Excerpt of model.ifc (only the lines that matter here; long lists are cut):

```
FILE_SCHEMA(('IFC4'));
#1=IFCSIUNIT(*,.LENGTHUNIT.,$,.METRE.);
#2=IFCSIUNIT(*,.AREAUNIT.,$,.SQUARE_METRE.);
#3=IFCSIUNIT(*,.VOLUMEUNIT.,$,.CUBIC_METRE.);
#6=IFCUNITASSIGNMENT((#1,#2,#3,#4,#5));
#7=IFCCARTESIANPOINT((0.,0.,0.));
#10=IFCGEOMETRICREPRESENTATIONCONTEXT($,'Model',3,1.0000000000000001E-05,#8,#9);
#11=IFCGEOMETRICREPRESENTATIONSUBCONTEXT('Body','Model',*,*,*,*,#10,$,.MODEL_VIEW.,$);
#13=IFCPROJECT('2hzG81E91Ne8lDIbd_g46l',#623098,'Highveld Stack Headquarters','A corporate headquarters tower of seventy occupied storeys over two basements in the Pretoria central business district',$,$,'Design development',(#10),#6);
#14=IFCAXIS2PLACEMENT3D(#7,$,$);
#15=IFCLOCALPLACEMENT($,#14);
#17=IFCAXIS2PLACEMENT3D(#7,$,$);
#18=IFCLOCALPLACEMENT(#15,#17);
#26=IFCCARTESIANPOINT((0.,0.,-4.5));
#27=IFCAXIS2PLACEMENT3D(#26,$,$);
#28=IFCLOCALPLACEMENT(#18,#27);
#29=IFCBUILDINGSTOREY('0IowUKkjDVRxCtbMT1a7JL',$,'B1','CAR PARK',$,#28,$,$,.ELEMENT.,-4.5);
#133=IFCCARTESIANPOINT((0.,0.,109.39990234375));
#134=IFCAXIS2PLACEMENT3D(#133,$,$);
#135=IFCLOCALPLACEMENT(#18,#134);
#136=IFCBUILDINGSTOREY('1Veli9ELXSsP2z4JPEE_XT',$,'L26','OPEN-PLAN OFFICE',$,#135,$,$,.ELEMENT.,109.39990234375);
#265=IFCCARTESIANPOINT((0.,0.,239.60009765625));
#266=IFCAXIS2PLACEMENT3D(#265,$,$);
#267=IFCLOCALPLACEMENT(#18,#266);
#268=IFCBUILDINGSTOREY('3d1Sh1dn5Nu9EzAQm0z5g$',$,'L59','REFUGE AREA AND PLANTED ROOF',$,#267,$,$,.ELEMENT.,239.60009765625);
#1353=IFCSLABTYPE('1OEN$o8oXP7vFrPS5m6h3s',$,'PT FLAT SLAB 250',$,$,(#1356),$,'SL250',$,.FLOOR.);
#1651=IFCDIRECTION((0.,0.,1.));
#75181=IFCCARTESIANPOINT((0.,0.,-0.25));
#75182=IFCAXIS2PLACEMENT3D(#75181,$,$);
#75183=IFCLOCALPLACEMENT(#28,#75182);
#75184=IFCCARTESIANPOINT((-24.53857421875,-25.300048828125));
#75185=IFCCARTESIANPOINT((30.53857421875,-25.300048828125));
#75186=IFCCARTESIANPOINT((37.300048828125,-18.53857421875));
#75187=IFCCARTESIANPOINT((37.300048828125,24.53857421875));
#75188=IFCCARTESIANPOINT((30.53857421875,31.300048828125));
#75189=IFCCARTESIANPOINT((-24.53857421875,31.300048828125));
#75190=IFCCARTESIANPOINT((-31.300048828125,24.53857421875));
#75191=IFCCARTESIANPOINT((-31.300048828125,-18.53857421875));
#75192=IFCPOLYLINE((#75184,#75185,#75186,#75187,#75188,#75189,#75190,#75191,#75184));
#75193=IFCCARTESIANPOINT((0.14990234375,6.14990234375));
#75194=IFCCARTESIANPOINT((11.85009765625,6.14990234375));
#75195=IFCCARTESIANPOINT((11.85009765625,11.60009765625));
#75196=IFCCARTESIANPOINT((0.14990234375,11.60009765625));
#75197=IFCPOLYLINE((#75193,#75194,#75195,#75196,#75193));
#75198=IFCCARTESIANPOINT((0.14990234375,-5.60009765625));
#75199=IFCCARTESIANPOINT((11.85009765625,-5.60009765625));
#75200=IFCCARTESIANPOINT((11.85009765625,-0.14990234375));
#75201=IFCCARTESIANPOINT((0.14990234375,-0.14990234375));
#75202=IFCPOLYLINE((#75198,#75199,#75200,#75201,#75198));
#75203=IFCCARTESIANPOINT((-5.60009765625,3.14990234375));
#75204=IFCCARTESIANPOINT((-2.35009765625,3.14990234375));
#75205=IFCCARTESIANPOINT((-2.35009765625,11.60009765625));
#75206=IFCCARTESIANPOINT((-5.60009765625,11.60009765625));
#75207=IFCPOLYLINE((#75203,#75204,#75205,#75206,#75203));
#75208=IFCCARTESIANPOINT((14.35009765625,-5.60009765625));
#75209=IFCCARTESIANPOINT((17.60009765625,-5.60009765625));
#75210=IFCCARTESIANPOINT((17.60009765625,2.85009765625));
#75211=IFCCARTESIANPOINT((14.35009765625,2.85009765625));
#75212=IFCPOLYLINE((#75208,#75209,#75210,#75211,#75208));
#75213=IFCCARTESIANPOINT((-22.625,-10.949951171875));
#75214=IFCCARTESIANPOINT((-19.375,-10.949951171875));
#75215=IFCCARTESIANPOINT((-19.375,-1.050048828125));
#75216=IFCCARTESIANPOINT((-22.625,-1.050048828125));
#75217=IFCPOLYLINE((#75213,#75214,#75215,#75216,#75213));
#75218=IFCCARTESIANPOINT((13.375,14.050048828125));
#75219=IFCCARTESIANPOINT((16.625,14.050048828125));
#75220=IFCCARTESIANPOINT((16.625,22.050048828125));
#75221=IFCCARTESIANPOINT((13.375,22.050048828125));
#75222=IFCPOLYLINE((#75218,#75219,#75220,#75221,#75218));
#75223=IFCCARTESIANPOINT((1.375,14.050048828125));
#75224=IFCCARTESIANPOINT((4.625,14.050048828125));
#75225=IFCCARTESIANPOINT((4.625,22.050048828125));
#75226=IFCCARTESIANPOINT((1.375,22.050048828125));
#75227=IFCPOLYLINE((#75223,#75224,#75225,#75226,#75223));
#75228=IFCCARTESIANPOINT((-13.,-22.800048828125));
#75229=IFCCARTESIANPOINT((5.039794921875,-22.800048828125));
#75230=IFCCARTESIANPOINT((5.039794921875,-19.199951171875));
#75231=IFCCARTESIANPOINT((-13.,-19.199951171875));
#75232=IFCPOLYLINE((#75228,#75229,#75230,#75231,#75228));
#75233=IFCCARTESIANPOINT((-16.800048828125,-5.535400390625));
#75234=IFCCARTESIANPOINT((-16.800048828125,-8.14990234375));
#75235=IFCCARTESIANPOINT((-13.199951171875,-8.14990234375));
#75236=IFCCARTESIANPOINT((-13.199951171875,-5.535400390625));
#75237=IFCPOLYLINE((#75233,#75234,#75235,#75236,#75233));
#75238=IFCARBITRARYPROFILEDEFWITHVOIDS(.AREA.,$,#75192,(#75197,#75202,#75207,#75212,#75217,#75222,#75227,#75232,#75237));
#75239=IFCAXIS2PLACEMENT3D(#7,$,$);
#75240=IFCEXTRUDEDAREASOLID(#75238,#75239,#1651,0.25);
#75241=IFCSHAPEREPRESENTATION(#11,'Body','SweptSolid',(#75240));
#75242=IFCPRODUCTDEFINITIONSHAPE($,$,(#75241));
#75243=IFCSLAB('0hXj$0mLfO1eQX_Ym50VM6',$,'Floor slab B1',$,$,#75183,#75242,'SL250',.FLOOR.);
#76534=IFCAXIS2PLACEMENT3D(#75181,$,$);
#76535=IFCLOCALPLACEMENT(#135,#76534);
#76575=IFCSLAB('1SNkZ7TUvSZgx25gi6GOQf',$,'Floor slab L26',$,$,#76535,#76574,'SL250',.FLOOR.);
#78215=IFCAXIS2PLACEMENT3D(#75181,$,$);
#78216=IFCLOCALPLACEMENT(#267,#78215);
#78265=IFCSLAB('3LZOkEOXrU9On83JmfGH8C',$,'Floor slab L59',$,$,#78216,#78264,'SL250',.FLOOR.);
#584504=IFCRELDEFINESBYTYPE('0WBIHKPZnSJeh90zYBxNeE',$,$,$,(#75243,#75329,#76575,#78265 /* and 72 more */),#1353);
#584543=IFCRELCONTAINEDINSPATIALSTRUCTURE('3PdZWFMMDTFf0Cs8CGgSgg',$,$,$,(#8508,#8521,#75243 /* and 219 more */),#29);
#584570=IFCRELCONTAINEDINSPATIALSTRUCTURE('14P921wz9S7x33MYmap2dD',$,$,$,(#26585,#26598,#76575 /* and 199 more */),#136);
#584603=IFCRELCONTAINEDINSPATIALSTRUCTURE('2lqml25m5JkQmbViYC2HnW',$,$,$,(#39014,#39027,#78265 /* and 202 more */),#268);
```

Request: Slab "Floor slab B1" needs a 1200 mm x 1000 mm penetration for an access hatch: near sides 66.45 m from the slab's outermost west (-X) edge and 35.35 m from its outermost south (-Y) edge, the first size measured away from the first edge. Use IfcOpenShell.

```python
import numpy as np
import ifcopenshell
import ifcopenshell.api.feature
import ifcopenshell.api.geometry
import ifcopenshell.api.root
import ifcopenshell.geom
import ifcopenshell.util.placement
import ifcopenshell.util.representation
import ifcopenshell.util.shape
import ifcopenshell.util.unit

model = ifcopenshell.open("model.ifc")
unit_scale = ifcopenshell.util.unit.calculate_unit_scale(model)
settings = ifcopenshell.geom.settings()


def volume(element):
    """Net volume in cubic metres, openings subtracted."""
    shape = ifcopenshell.geom.create_shape(settings, element)
    return ifcopenshell.util.shape.get_volume(shape.geometry)


slab = model.by_guid("0hXj$0mLfO1eQX_Ym50VM6")
before = volume(slab)

# Extent in the slab's own axes, in metres. The edges named are its -X and -Y sides.
slab_shape = ifcopenshell.geom.create_shape(settings, slab)
vertices = ifcopenshell.util.shape.get_vertices(slab_shape.geometry)
x_min, y_min, bottom = vertices.min(axis=0)
top = vertices[:, 2].max()

opening = ifcopenshell.api.root.create_entity(model, ifc_class="IfcOpeningElement", name="Access hatch opening", predefined_type="OPENING")
context = ifcopenshell.util.representation.get_context(model, "Model", "Body", "MODEL_VIEW")
width, depth = 1.2, 1
outline = [(0.0, 0.0), (width, 0.0), (width, depth), (0.0, depth), (0.0, 0.0)]
# Overshoot both faces by 50 mm so the cut is clean.
shape = ifcopenshell.api.geometry.add_slab_representation(
    model, context=context, depth=top - bottom + 0.1, polyline=outline
)
ifcopenshell.api.geometry.assign_representation(model, product=opening, representation=shape)

matrix = ifcopenshell.util.placement.get_local_placement(slab.ObjectPlacement)
matrix[:, 3] = matrix @ np.append(np.array([x_min + 66.45, y_min + 35.35, bottom - 0.05]) / unit_scale, 1.0)
ifcopenshell.api.geometry.edit_object_placement(model, product=opening, matrix=matrix, is_si=False)
ifcopenshell.api.feature.add_feature(model, feature=opening, element=slab)

after = volume(slab)

print(f"slab volume {before:.3f} -> {after:.3f} m3")

model.write("model_v2.ifc")
```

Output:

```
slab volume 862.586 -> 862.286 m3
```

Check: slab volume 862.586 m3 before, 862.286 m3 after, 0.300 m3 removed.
